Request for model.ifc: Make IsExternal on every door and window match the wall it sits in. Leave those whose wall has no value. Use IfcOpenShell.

First a look at what the model holds.

```python
import ifcopenshell
import ifcopenshell.util.element

model = ifcopenshell.open("model.ifc")
print(model.schema)
seen = {}
for e in model.by_type("IfcDoor") + model.by_type("IfcWindow"):
    if not e.FillsVoids:
        continue
    host = e.FillsVoids[0].RelatingOpeningElement.VoidsElements[0].RelatingBuildingElement
    own = ifcopenshell.util.element.get_pset(e, f"Pset_{e.is_a()[3:].removesuffix('StandardCase')}Common", "IsExternal")
    wall = ifcopenshell.util.element.get_pset(host, "Pset_WallCommon", "IsExternal")
    seen[e.is_a(), own, wall] = seen.get((e.is_a(), own, wall), 0) + 1
for (cls, own, wall), count in sorted(seen.items(), key=str):
    print(count, cls, "IsExternal:", own, "| host wall:", wall)
```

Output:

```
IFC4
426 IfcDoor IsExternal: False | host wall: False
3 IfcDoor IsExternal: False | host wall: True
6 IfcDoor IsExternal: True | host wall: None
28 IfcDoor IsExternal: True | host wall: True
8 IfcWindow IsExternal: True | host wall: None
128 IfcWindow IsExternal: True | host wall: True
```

```python
import ifcopenshell
import ifcopenshell.api.pset
import ifcopenshell.util.element

model = ifcopenshell.open("model.ifc")

count = 0
for ifc_class, pset_name in (("IfcDoor", "Pset_DoorCommon"), ("IfcWindow", "Pset_WindowCommon")):
    for e in model.by_type(ifc_class):
        if not e.FillsVoids:
            continue
        host = e.FillsVoids[0].RelatingOpeningElement.VoidsElements[0].RelatingBuildingElement
        external = ifcopenshell.util.element.get_pset(host, "Pset_WallCommon", "IsExternal")
        if external is None or ifcopenshell.util.element.get_pset(e, pset_name, "IsExternal") == external:
            continue
        pset = ifcopenshell.api.pset.add_pset(model, product=e, name=pset_name)
        ifcopenshell.api.pset.edit_pset(model, pset=pset, properties={"IsExternal": external})
        count += 1

print(count, "updated")

model.write("model_edited.ifc")
```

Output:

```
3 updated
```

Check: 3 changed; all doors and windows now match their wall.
